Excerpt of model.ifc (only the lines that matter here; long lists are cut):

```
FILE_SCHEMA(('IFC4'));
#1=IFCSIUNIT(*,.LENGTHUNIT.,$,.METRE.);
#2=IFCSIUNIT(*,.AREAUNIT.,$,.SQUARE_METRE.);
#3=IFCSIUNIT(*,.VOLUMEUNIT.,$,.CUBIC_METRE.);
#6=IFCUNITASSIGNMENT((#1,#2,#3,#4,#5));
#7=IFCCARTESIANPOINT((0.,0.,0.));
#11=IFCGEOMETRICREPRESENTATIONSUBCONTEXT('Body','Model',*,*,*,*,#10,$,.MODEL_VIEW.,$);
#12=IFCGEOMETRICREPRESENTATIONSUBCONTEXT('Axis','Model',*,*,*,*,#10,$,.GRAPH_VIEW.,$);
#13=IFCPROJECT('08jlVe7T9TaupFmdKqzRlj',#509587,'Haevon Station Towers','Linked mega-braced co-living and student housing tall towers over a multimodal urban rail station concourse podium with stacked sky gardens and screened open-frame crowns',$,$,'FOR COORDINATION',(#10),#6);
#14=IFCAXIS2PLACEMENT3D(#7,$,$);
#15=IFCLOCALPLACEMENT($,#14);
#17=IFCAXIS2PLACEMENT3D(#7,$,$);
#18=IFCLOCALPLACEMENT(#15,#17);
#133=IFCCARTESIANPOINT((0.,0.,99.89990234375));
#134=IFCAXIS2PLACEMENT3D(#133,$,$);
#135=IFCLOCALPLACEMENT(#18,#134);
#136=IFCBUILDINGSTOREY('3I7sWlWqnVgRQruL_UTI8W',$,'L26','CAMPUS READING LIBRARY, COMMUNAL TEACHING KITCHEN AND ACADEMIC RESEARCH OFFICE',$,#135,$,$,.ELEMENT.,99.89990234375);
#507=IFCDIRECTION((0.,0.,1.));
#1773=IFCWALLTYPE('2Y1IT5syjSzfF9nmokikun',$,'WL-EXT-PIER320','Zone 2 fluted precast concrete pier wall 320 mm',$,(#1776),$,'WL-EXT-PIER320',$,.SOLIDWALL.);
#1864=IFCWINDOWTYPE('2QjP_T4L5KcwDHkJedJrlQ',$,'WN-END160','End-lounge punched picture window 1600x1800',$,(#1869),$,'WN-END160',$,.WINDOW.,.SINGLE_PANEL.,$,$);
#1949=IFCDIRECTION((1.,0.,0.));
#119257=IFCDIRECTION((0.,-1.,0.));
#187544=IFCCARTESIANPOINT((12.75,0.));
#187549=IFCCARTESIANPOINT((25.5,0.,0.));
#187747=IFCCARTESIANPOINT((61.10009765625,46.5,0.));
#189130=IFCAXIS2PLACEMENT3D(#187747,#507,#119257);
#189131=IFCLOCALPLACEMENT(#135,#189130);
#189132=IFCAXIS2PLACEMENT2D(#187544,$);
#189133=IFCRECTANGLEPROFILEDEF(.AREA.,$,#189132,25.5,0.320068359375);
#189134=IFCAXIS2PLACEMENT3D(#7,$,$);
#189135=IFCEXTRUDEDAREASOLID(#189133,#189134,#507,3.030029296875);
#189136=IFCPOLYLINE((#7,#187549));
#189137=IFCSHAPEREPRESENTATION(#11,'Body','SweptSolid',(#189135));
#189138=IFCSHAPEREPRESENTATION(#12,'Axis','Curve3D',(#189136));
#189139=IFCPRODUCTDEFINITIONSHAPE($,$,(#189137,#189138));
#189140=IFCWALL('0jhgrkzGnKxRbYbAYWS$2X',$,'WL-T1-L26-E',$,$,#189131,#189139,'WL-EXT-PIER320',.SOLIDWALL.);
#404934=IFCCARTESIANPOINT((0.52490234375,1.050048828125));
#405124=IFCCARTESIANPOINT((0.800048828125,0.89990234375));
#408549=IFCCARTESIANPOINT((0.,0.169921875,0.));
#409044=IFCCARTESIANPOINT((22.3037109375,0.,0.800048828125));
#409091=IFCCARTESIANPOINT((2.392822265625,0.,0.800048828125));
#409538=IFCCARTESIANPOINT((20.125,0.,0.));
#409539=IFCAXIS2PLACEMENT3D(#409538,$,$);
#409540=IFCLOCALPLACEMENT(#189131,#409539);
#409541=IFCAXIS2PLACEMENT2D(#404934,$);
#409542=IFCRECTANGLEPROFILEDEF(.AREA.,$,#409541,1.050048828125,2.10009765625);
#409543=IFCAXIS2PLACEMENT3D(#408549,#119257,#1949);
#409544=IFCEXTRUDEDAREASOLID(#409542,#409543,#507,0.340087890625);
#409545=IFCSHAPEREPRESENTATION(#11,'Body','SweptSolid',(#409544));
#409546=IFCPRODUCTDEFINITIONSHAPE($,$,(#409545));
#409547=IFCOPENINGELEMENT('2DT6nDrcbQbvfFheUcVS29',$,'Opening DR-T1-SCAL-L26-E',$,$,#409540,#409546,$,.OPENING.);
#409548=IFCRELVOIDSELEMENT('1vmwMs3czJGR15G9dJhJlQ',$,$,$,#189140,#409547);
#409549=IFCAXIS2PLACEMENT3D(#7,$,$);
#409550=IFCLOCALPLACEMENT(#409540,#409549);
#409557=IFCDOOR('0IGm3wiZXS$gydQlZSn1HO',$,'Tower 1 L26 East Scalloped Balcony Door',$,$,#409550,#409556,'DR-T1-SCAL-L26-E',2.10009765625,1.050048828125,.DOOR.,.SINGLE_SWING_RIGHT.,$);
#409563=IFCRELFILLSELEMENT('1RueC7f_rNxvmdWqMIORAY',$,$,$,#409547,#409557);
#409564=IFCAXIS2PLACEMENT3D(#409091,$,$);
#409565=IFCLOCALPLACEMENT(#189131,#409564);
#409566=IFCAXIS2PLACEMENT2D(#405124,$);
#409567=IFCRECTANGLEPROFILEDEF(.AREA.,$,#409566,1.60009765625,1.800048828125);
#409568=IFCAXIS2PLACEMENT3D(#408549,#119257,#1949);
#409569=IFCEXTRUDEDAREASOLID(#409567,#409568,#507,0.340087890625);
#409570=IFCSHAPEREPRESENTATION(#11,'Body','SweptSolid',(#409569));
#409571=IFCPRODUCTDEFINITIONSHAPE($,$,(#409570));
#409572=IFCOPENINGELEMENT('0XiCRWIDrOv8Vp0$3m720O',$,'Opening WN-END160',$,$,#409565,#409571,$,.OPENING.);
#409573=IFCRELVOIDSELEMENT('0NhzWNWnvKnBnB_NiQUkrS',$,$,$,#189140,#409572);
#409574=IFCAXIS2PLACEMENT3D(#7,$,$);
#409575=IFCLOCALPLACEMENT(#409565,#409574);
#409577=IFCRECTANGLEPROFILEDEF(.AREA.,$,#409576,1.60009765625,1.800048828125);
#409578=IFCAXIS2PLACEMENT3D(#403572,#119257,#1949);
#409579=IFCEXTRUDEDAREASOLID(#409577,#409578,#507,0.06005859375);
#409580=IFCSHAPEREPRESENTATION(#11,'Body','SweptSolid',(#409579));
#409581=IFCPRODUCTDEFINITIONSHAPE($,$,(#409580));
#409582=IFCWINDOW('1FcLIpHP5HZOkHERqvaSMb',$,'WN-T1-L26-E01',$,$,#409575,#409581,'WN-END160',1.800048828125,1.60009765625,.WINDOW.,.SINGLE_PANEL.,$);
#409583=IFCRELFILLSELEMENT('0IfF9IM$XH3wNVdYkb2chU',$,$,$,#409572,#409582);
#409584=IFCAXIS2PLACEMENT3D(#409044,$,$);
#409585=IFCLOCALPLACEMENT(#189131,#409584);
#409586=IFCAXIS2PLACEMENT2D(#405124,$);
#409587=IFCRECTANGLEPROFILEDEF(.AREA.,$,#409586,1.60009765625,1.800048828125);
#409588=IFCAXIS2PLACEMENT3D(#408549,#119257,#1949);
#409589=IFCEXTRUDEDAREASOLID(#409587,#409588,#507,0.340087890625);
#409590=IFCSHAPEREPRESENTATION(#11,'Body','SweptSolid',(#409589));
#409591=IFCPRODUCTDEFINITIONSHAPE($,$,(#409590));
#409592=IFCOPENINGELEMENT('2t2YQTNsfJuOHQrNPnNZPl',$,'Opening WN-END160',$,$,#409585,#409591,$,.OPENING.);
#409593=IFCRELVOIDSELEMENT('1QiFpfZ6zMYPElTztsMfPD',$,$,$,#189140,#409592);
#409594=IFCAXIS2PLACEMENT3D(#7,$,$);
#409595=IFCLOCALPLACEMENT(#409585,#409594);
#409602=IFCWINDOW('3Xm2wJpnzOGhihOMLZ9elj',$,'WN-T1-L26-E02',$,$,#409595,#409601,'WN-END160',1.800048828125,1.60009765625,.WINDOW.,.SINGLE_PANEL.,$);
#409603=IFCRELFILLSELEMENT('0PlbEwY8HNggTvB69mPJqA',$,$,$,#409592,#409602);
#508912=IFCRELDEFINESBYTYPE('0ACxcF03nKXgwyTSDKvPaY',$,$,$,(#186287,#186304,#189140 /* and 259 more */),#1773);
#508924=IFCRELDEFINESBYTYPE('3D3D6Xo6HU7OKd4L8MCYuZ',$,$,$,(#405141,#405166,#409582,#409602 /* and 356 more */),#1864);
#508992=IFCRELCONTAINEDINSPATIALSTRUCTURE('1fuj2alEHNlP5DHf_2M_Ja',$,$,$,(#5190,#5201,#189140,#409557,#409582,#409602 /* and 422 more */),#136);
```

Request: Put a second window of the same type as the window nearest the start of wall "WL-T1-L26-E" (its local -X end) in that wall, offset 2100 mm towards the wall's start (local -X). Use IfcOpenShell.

```python
import ifcopenshell
import ifcopenshell.api.feature
import ifcopenshell.api.geometry
import ifcopenshell.api.root
import ifcopenshell.geom
import ifcopenshell.util.element
import ifcopenshell.util.placement
import ifcopenshell.util.shape
import ifcopenshell.util.unit

model = ifcopenshell.open("model.ifc")
unit_scale = ifcopenshell.util.unit.calculate_unit_scale(model)
settings = ifcopenshell.geom.settings()


def volume(element):
    """Net volume in cubic metres, openings subtracted."""
    shape = ifcopenshell.geom.create_shape(settings, element)
    return ifcopenshell.util.shape.get_volume(shape.geometry)


window = model.by_guid("1FcLIpHP5HZOkHERqvaSMb")
opening = window.FillsVoids[0].RelatingOpeningElement
wall = opening.VoidsElements[0].RelatingBuildingElement
before = volume(wall)
shift = ifcopenshell.util.placement.get_local_placement(wall.ObjectPlacement)[:3, 0] * -2.1 / unit_scale

# copy_class copies the void relationship, type, container and properties, but no geometry.
new_opening = ifcopenshell.api.root.copy_class(model, product=opening)
new_opening.Representation = ifcopenshell.util.element.copy_deep(
    model, opening.Representation, exclude=["IfcGeometricRepresentationContext", "IfcRepresentationMap"]
)
new_window = ifcopenshell.api.root.copy_class(model, product=window)
new_window.Representation = ifcopenshell.util.element.copy_deep(
    model, window.Representation, exclude=["IfcGeometricRepresentationContext", "IfcRepresentationMap"]
)
new_window.Tag = None
ifcopenshell.api.feature.add_filling(model, opening=new_opening, element=new_window)

for old, new in ((opening, new_opening), (window, new_window)):
    matrix = ifcopenshell.util.placement.get_local_placement(old.ObjectPlacement)
    matrix[:3, 3] += shift
    ifcopenshell.api.geometry.edit_object_placement(model, product=new, matrix=matrix, is_si=False)

after = volume(wall)

print(f"wall volume {before:.3f} -> {after:.3f} m3")

model.write("model_v2.ifc")
```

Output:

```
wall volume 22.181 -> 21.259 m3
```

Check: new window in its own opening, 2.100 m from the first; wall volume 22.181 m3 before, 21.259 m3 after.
